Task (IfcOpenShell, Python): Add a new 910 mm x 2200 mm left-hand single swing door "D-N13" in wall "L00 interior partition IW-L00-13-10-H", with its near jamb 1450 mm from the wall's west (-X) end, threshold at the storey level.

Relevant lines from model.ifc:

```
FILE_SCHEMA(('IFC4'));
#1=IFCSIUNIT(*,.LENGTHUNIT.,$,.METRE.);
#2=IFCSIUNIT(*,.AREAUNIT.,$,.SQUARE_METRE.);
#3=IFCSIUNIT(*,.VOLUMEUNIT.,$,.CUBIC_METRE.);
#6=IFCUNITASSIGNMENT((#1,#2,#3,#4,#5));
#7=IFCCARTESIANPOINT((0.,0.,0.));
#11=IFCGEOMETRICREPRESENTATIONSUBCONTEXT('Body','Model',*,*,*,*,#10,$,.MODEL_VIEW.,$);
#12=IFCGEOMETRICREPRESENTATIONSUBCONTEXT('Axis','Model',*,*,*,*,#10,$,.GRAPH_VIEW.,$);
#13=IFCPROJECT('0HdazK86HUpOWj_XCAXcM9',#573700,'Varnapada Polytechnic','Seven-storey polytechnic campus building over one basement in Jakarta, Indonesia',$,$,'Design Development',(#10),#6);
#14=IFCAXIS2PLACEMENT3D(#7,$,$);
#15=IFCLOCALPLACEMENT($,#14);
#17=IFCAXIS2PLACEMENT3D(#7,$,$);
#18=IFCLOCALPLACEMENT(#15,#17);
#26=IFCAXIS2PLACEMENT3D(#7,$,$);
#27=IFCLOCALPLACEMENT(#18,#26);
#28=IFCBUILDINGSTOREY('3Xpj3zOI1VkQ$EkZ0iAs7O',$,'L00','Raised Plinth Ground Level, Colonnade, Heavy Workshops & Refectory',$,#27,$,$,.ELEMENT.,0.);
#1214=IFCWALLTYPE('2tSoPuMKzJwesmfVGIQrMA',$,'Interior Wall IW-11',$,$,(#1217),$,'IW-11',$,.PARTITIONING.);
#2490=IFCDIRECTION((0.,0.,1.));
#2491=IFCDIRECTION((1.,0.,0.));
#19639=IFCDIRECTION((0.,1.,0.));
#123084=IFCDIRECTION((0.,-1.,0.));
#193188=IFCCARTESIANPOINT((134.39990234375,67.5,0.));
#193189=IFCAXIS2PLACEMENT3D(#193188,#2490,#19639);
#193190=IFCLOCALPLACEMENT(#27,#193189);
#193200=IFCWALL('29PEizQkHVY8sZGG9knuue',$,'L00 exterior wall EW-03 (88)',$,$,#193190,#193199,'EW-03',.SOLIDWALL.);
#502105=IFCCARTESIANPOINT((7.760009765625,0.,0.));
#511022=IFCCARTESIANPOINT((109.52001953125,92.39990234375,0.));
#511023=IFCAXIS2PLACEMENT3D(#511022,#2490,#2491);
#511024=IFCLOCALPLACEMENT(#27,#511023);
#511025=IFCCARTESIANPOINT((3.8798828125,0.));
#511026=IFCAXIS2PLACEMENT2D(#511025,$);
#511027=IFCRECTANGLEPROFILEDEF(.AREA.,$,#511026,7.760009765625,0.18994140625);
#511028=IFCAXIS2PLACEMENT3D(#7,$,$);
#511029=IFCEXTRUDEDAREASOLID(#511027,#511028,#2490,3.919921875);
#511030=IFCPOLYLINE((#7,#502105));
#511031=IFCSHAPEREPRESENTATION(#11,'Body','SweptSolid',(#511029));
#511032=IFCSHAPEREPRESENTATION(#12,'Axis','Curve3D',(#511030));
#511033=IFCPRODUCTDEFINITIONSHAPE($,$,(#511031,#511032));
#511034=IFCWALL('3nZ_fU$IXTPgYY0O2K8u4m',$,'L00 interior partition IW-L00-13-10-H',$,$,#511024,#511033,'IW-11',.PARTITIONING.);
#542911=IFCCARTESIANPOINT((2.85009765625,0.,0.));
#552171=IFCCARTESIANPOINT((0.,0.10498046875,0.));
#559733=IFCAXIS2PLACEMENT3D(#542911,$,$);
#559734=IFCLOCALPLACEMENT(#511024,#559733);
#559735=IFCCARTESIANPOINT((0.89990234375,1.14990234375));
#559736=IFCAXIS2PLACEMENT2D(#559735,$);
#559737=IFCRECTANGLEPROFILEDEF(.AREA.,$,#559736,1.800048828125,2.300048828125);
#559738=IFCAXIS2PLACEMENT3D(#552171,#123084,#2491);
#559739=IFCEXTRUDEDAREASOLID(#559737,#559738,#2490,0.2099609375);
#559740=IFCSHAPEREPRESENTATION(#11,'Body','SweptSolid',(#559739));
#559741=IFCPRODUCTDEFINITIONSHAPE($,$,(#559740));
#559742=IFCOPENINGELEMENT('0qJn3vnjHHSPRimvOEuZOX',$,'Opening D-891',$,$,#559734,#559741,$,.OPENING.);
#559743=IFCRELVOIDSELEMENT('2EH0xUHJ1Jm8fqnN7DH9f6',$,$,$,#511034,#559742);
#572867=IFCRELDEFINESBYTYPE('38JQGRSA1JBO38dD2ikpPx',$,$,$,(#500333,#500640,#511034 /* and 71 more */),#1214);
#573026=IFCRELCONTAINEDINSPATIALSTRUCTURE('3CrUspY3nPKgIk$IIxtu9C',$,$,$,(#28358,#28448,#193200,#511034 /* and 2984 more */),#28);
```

```python
import numpy as np
import ifcopenshell
import ifcopenshell.api.feature
import ifcopenshell.api.geometry
import ifcopenshell.api.root
import ifcopenshell.api.spatial
import ifcopenshell.geom
import ifcopenshell.util.element
import ifcopenshell.util.placement
import ifcopenshell.util.representation
import ifcopenshell.util.shape
import ifcopenshell.util.unit

model = ifcopenshell.open("model.ifc")
unit_scale = ifcopenshell.util.unit.calculate_unit_scale(model)
settings = ifcopenshell.geom.settings()


def volume(element):
    """Net volume in cubic metres, openings subtracted."""
    shape = ifcopenshell.geom.create_shape(settings, element)
    return ifcopenshell.util.shape.get_volume(shape.geometry)


wall = model.by_guid("3nZ_fU$IXTPgYY0O2K8u4m")
storey = ifcopenshell.util.element.get_container(wall, ifc_class="IfcBuildingStorey")
context = ifcopenshell.util.representation.get_context(model, "Model", "Body", "MODEL_VIEW")
before = volume(wall)

width, height, from_end, sill = 0.91, 2.2, 1.45, 0.0  # metres

# The wall runs along its own X axis, and the end named is its -X end.
wall_shape = ifcopenshell.geom.create_shape(settings, wall)
x, y, z = ifcopenshell.util.shape.get_vertices(wall_shape.geometry).T
start = x.min() + from_end
face, thickness = float(y.min()), float(y.max() - y.min())
wall_matrix = ifcopenshell.util.placement.get_local_placement(wall.ObjectPlacement)
level = ifcopenshell.util.placement.get_local_placement(storey.ObjectPlacement)[2, 3]


def in_wall(x, y):
    """Placement at x, y metres in the wall's axes, at sill height."""
    matrix = wall_matrix.copy()
    matrix[:, 3] = wall_matrix @ np.array([x / unit_scale, y / unit_scale, 0.0, 1.0])
    matrix[2, 3] = level + sill / unit_scale
    return matrix


# Opening: a box that overshoots both wall faces by 50 mm.
opening = ifcopenshell.api.root.create_entity(model, ifc_class="IfcOpeningElement", predefined_type="OPENING")
box = ifcopenshell.api.geometry.add_wall_representation(
    model, context=context, length=width, height=height, thickness=thickness + 0.1
)
ifcopenshell.api.geometry.assign_representation(model, product=opening, representation=box)
ifcopenshell.api.geometry.edit_object_placement(model, product=opening, matrix=in_wall(start, face - 0.05), is_si=False)
ifcopenshell.api.feature.add_feature(model, feature=opening, element=wall)

door = ifcopenshell.api.root.create_entity(model, ifc_class="IfcDoor", name="D-N13", predefined_type="DOOR")
door.OverallWidth, door.OverallHeight = width / unit_scale, height / unit_scale
door.OperationType = "SINGLE_SWING_LEFT"
body = ifcopenshell.api.geometry.add_door_representation(
    model,
    context=context,
    overall_width=door.OverallWidth,
    overall_height=door.OverallHeight,
    operation_type="SINGLE_SWING_LEFT",
    lining_properties={"LiningDepth": thickness / unit_scale, "ThresholdDepth": thickness / unit_scale},
)
ifcopenshell.api.geometry.assign_representation(model, product=door, representation=body)
ifcopenshell.api.spatial.assign_container(model, products=[door], relating_structure=storey)
ifcopenshell.api.feature.add_filling(model, opening=opening, element=door)

# The lining spans the wall, so the door starts at the wall face.
ifcopenshell.api.geometry.edit_object_placement(model, product=door, matrix=in_wall(start, face), is_si=False)

after = volume(wall)

print(f"wall volume {before:.3f} -> {after:.3f} m3")

model.write("model_v2.ifc")
```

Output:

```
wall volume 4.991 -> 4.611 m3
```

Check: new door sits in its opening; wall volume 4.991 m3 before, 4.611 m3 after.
